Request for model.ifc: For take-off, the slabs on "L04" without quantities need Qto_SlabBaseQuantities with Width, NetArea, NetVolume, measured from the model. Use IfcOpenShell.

First a look at what the model holds.

```python
import ifcopenshell
import ifcopenshell.util.element
import ifcopenshell.util.unit

model = ifcopenshell.open("model.ifc")
print(model.schema)
for unit_type in ("LENGTHUNIT", "AREAUNIT", "VOLUMEUNIT"):
    print(unit_type, ifcopenshell.util.unit.calculate_unit_scale(model, unit_type))
storey = next(s for s in model.by_type("IfcBuildingStorey") if s.Name == "L04")
slabs = [e for e in ifcopenshell.util.element.get_decomposition(storey) if e.is_a("IfcSlab")]
for e in sorted(slabs, key=lambda e: e.id()):
    print(e.id(), e.is_a(), e.Name, list(ifcopenshell.util.element.get_psets(e, qtos_only=True)), sep=" | ")
```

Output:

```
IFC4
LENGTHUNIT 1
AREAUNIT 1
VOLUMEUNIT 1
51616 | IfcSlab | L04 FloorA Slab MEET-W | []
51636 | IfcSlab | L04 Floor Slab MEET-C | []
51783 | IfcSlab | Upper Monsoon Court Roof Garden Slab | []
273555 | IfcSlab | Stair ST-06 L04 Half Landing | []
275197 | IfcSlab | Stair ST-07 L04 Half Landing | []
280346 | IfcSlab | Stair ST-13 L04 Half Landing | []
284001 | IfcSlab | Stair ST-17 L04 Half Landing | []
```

```python
import ifcopenshell
import ifcopenshell.api.pset
import ifcopenshell.geom
import ifcopenshell.util.element
import ifcopenshell.util.shape
import ifcopenshell.util.unit

model = ifcopenshell.open("model.ifc")
unit_scale = ifcopenshell.util.unit.calculate_unit_scale(model)
area_scale = ifcopenshell.util.unit.calculate_unit_scale(model, "AREAUNIT")
volume_scale = ifcopenshell.util.unit.calculate_unit_scale(model, "VOLUMEUNIT")
settings = ifcopenshell.geom.settings()

storey = next(s for s in model.by_type("IfcBuildingStorey") if s.Name == "L04")
slabs = [e for e in ifcopenshell.util.element.get_decomposition(storey) if e.is_a("IfcSlab")]

for e in sorted(slabs, key=lambda e: e.id()):
    if ifcopenshell.util.element.get_psets(e, qtos_only=True, should_inherit=False):
        continue
    # Geometry comes back in metres, in the element's own axes.
    shape = ifcopenshell.geom.create_shape(settings, e)
    values = {
        "Width": ifcopenshell.util.shape.get_z(shape.geometry) / unit_scale,
        "NetArea": ifcopenshell.util.shape.get_footprint_area(shape.geometry) / area_scale,
        "NetVolume": ifcopenshell.util.shape.get_volume(shape.geometry) / volume_scale,
    }
    qto = ifcopenshell.api.pset.add_qto(model, product=e, name="Qto_SlabBaseQuantities")
    ifcopenshell.api.pset.edit_qto(model, qto=qto, properties=values)
    print(e.id(), {k: round(v, 3) for k, v in values.items()})

model.write("model-out.ifc")
```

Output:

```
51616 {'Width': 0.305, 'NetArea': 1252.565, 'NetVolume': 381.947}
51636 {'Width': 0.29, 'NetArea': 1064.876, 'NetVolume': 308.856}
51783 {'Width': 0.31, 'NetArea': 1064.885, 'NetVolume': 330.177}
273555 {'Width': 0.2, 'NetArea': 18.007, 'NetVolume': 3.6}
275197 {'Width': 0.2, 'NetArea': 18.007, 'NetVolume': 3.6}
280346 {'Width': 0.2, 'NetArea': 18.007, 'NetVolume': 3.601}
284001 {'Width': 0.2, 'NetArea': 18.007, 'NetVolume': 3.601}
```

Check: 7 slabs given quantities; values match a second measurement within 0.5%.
